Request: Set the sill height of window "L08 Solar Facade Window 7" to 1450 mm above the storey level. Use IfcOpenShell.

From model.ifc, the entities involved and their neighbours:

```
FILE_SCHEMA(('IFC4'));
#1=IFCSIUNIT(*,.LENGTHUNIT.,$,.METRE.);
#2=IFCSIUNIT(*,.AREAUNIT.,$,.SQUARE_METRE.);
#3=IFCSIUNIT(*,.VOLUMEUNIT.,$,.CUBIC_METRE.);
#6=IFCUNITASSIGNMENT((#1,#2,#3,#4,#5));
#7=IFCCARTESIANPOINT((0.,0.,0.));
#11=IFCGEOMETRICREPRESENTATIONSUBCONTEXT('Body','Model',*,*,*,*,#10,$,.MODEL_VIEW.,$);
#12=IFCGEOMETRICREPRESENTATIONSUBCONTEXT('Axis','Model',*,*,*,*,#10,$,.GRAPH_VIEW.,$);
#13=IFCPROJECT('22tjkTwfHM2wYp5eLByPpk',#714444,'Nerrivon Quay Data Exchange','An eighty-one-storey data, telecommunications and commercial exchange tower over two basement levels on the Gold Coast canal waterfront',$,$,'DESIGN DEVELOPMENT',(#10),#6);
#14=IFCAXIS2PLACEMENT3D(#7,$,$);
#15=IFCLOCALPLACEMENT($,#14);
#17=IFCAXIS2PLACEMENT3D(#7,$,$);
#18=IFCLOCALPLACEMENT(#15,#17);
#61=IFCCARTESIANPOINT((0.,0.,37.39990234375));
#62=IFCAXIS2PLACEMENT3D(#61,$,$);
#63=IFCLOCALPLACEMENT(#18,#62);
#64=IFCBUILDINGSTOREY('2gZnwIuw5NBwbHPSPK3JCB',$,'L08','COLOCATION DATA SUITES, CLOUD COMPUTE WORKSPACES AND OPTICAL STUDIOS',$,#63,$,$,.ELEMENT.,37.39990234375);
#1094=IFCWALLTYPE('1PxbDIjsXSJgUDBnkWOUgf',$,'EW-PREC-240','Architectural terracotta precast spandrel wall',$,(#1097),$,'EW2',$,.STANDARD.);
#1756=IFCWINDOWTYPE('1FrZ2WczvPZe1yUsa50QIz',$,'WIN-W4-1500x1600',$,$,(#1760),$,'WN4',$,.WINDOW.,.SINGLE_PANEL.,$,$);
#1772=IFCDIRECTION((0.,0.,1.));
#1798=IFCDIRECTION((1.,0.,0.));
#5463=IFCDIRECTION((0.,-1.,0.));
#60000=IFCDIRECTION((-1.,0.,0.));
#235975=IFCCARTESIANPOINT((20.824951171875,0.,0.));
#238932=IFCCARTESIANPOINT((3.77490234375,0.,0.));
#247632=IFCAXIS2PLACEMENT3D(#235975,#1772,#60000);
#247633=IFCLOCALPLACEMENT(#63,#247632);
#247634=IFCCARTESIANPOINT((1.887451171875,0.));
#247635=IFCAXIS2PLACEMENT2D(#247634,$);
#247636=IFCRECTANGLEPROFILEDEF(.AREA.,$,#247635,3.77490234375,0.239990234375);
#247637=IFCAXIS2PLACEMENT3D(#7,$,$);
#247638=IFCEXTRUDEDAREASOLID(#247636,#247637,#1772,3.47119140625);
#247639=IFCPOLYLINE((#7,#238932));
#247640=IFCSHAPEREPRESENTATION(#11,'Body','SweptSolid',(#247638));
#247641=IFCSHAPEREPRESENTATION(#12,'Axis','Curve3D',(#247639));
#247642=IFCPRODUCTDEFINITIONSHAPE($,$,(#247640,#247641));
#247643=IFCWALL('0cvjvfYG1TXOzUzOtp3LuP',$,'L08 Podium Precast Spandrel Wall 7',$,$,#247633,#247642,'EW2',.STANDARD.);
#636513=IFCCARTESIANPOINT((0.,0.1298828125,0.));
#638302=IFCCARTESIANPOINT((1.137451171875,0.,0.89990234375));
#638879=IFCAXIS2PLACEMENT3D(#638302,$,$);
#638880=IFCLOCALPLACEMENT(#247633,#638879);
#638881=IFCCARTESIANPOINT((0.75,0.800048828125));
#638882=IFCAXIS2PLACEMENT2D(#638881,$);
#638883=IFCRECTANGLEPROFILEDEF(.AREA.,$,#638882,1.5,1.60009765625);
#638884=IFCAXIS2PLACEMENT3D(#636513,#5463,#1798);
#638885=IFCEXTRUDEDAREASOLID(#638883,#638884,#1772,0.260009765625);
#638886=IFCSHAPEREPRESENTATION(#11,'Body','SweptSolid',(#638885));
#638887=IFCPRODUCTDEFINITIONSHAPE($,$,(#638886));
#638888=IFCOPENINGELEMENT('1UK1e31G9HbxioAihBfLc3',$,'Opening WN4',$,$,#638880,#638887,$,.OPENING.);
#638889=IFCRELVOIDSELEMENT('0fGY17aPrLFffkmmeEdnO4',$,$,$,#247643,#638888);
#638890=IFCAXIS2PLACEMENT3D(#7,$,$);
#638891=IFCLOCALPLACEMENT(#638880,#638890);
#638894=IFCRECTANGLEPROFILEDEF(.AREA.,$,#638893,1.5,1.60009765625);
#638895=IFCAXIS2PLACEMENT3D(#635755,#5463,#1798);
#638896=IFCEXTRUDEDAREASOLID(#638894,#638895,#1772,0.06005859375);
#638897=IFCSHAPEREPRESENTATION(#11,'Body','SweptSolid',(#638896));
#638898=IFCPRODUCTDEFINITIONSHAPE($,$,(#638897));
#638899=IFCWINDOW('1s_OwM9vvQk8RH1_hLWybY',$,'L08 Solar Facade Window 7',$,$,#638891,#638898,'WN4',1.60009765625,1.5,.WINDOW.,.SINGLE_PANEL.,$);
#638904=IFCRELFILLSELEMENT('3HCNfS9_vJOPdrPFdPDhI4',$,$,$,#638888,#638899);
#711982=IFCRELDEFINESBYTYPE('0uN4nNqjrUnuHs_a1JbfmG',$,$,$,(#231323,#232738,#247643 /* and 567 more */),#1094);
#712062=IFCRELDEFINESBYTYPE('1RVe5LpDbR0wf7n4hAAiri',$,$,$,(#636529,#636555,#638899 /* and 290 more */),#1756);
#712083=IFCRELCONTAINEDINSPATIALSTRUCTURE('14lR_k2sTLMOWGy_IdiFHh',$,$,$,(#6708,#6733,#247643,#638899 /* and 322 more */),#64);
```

```python
import numpy as np
import ifcopenshell
import ifcopenshell.api.geometry
import ifcopenshell.geom
import ifcopenshell.util.element
import ifcopenshell.util.placement
import ifcopenshell.util.shape
import ifcopenshell.util.unit

model = ifcopenshell.open("model.ifc")
unit_scale = ifcopenshell.util.unit.calculate_unit_scale(model)

window = model.by_guid("1s_OwM9vvQk8RH1_hLWybY")
opening = window.FillsVoids[0].RelatingOpeningElement
storey = ifcopenshell.util.element.get_container(window, ifc_class="IfcBuildingStorey")
level = ifcopenshell.util.placement.get_local_placement(storey.ObjectPlacement)[2, 3]

# The opening's origin need not be at the sill, so measure its lowest point.
shape = ifcopenshell.geom.create_shape(ifcopenshell.geom.settings(), opening)
bottom = ifcopenshell.util.shape.get_shape_bottom_elevation(shape, shape.geometry) / unit_scale
dz = level + 1.45 / unit_scale - bottom

shift = np.array([0.0, 0.0, dz])
# The window is placed relative to its opening, so it follows when the opening moves.
matrix = ifcopenshell.util.placement.get_local_placement(opening.ObjectPlacement)
matrix[:3, 3] += shift
ifcopenshell.api.geometry.edit_object_placement(
    model, product=opening, matrix=matrix, is_si=False, should_transform_children=True
)

print(f"moved by {dz * unit_scale:+.3f} m")

model.write("model_v2.ifc")
```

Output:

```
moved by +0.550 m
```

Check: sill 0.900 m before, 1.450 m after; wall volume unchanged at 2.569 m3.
